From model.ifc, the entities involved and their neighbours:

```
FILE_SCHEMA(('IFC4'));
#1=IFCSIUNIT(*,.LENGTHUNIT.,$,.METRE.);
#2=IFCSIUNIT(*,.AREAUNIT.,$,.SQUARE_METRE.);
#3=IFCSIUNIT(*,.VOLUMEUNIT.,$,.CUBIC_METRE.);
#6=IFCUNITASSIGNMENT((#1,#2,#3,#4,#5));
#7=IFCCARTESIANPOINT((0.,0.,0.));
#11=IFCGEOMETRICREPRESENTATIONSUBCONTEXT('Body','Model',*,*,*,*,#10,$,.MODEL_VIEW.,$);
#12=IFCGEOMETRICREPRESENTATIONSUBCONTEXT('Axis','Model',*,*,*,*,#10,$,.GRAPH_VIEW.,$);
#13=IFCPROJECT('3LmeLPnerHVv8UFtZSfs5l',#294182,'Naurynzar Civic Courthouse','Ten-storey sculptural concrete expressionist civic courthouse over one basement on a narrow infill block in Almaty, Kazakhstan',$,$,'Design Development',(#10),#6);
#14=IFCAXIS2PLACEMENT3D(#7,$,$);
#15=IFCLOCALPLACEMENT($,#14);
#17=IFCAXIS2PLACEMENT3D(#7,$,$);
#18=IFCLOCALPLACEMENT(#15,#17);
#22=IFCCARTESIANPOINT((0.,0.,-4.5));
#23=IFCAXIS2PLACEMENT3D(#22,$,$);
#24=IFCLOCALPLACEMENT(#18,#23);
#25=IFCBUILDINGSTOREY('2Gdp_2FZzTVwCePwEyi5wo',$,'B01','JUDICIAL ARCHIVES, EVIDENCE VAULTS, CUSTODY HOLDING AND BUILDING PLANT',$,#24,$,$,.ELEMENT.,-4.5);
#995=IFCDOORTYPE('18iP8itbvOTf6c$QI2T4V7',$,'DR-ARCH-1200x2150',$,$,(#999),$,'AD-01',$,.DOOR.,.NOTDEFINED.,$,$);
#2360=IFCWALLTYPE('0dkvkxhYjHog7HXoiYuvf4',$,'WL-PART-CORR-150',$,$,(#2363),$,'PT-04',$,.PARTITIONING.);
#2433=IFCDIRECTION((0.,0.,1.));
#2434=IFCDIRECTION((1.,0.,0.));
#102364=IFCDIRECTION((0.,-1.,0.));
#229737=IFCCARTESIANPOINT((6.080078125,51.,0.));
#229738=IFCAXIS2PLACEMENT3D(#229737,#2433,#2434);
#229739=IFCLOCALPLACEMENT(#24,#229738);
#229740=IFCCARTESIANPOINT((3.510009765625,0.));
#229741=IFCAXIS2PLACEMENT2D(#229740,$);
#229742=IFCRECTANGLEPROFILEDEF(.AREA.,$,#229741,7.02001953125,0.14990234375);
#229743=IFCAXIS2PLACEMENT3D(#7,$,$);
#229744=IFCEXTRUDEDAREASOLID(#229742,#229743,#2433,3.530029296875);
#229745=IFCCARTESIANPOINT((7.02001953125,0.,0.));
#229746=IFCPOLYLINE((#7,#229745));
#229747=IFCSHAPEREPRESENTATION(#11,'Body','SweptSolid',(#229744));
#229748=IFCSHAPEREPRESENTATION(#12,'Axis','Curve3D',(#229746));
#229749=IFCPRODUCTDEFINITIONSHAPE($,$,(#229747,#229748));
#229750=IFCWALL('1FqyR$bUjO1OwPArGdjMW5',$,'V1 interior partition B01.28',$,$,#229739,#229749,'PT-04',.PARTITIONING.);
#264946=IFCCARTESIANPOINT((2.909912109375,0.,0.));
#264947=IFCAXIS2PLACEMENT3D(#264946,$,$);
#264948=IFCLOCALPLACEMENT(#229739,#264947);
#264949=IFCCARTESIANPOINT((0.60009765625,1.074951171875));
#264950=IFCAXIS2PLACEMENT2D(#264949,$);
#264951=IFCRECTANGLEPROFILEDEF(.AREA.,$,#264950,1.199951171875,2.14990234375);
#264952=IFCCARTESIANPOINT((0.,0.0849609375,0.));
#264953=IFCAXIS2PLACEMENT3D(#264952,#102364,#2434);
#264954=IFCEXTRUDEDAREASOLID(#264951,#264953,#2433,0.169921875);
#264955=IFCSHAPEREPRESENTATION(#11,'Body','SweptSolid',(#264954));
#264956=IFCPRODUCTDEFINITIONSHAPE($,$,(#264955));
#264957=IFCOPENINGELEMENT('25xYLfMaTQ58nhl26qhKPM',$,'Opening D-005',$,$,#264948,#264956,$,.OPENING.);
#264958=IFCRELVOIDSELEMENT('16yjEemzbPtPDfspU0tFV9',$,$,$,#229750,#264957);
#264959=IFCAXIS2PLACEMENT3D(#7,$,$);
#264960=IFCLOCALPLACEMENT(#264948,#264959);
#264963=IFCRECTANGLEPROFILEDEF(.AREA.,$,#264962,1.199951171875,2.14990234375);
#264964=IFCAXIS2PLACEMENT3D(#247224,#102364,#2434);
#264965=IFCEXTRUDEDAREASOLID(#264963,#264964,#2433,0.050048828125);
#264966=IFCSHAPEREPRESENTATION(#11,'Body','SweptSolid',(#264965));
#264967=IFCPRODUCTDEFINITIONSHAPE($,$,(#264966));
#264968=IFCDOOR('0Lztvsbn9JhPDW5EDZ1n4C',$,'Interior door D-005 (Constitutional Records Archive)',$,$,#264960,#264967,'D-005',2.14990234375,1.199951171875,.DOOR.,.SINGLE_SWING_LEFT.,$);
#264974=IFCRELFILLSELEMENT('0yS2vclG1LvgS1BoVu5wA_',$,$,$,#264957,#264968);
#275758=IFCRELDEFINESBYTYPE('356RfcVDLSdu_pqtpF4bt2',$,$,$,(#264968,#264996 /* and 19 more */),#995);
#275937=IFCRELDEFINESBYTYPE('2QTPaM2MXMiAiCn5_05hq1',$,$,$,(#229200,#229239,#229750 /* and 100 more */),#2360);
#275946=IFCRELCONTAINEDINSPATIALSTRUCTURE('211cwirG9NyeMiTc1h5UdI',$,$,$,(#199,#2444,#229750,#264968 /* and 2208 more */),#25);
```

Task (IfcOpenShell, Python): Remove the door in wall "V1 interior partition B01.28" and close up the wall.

```python
import ifcopenshell
import ifcopenshell.api.feature
import ifcopenshell.api.root
import ifcopenshell.geom
import ifcopenshell.util.shape

model = ifcopenshell.open("model.ifc")
settings = ifcopenshell.geom.settings()


def volume(element):
    """Net volume in cubic metres, openings subtracted."""
    shape = ifcopenshell.geom.create_shape(settings, element)
    return ifcopenshell.util.shape.get_volume(shape.geometry)


door = model.by_guid("0Lztvsbn9JhPDW5EDZ1n4C")
opening = door.FillsVoids[0].RelatingOpeningElement
wall = opening.VoidsElements[0].RelatingBuildingElement
before = volume(wall)

ifcopenshell.api.root.remove_product(model, product=door)
ifcopenshell.api.feature.remove_feature(model, feature=opening)

after = volume(wall)

print(f"wall volume {before:.3f} -> {after:.3f} m3")

model.write("model_rev.ifc")
```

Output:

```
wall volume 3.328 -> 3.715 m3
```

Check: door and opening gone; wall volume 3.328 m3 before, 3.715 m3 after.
